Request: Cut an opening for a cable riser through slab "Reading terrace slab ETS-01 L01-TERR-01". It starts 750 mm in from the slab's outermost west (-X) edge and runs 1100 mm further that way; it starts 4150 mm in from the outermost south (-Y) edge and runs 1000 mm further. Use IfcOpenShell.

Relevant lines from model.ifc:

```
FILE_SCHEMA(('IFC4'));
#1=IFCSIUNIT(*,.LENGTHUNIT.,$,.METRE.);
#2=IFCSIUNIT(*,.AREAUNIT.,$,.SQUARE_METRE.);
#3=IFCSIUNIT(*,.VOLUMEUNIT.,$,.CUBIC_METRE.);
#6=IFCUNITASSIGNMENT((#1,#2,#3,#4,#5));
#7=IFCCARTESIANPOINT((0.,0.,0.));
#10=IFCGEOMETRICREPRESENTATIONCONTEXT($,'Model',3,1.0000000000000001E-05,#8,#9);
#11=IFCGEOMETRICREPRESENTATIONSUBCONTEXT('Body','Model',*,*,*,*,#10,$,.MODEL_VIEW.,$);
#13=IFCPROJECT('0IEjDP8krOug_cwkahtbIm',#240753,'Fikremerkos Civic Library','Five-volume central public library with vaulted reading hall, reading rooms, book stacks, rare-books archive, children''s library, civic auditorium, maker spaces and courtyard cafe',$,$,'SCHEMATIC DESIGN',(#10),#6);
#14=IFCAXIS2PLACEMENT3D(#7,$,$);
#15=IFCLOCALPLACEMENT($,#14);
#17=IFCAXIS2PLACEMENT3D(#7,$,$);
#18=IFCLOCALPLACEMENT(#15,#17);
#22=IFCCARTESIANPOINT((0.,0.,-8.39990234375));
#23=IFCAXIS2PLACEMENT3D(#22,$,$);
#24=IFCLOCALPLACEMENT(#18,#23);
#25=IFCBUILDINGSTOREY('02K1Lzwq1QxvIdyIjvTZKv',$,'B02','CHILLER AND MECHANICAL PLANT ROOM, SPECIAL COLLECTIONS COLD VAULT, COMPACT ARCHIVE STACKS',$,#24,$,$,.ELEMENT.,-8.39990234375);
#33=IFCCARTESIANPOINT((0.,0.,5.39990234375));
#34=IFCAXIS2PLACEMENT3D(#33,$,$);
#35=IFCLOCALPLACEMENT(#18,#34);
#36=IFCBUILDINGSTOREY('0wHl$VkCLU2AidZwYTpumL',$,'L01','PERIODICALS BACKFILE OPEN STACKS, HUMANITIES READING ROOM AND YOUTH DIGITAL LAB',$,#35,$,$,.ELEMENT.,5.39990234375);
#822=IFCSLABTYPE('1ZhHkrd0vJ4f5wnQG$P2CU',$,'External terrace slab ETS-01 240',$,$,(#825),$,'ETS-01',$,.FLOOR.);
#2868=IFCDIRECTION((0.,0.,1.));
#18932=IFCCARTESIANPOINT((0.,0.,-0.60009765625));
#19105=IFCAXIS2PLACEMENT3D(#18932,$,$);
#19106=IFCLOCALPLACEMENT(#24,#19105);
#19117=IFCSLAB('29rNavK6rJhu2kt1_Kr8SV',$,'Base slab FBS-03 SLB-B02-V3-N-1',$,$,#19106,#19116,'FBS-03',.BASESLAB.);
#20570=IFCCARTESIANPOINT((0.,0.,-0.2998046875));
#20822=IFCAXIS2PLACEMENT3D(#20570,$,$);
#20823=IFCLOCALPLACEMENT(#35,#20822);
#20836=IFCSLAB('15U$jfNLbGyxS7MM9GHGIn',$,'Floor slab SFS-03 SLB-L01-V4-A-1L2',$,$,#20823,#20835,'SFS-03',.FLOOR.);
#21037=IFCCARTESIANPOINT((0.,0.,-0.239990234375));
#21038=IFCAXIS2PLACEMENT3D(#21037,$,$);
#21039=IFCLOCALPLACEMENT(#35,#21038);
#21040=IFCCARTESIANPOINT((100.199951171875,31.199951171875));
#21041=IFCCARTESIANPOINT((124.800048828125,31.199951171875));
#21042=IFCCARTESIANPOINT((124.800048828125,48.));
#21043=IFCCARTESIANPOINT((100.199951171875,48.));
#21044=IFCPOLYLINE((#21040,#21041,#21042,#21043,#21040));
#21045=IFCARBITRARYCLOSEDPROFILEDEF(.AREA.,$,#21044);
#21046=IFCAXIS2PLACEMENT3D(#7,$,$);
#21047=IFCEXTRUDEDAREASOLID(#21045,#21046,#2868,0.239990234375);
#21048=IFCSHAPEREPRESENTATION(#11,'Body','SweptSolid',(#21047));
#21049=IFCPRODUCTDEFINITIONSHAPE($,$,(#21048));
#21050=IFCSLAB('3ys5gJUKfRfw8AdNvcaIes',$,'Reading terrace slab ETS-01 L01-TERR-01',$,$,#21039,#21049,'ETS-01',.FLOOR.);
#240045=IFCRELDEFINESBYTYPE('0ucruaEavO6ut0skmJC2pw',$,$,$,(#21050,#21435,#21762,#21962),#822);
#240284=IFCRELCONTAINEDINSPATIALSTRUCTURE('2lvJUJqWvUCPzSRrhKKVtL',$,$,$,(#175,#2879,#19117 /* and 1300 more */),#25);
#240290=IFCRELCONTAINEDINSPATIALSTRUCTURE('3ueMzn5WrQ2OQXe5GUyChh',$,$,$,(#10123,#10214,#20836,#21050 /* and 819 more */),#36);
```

```python
import numpy as np
import ifcopenshell
import ifcopenshell.api.feature
import ifcopenshell.api.geometry
import ifcopenshell.api.root
import ifcopenshell.geom
import ifcopenshell.util.placement
import ifcopenshell.util.representation
import ifcopenshell.util.shape
import ifcopenshell.util.unit

model = ifcopenshell.open("model.ifc")
unit_scale = ifcopenshell.util.unit.calculate_unit_scale(model)
settings = ifcopenshell.geom.settings()


def volume(element):
    """Net volume in cubic metres, openings subtracted."""
    shape = ifcopenshell.geom.create_shape(settings, element)
    return ifcopenshell.util.shape.get_volume(shape.geometry)


slab = model.by_guid("3ys5gJUKfRfw8AdNvcaIes")
before = volume(slab)

# Extent in the slab's own axes, in metres. The edges named are its -X and -Y sides.
slab_shape = ifcopenshell.geom.create_shape(settings, slab)
vertices = ifcopenshell.util.shape.get_vertices(slab_shape.geometry)
x_min, y_min, bottom = vertices.min(axis=0)
top = vertices[:, 2].max()

opening = ifcopenshell.api.root.create_entity(model, ifc_class="IfcOpeningElement", name="Cable riser opening", predefined_type="OPENING")
context = ifcopenshell.util.representation.get_context(model, "Model", "Body", "MODEL_VIEW")
width, depth = 1.1, 1
outline = [(0.0, 0.0), (width, 0.0), (width, depth), (0.0, depth), (0.0, 0.0)]
# Overshoot both faces by 50 mm so the cut is clean.
shape = ifcopenshell.api.geometry.add_slab_representation(
    model, context=context, depth=top - bottom + 0.1, polyline=outline
)
ifcopenshell.api.geometry.assign_representation(model, product=opening, representation=shape)

matrix = ifcopenshell.util.placement.get_local_placement(slab.ObjectPlacement)
matrix[:, 3] = matrix @ np.append(np.array([x_min + 0.75, y_min + 4.15, bottom - 0.05]) / unit_scale, 1.0)
ifcopenshell.api.geometry.edit_object_placement(model, product=opening, matrix=matrix, is_si=False)
ifcopenshell.api.feature.add_feature(model, feature=opening, element=slab)

after = volume(slab)

print(f"slab volume {before:.3f} -> {after:.3f} m3")

model.write("model_v2.ifc")
```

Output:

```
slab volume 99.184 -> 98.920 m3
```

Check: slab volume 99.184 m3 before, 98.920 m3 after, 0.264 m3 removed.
